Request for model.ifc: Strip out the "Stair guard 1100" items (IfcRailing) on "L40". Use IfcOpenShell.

First a look at what the model holds.

```python
import ifcopenshell
import ifcopenshell.util.element

model = ifcopenshell.open("model.ifc")
print(model.schema)
storey = next(s for s in model.by_type("IfcBuildingStorey") if s.Name == "L40")
railings = [e for e in ifcopenshell.util.element.get_decomposition(storey) if e.is_a("IfcRailing")]
seen = {}
for e in railings:
    element_type = ifcopenshell.util.element.get_type(e)
    name = element_type.Name if element_type not in (None, e) else None
    seen[name] = seen.get(name, 0) + 1
for name, count in sorted(seen.items(), key=str):
    print(count, "x", name)
```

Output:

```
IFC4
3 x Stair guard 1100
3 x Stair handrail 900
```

```python
import ifcopenshell
import ifcopenshell.api.root
import ifcopenshell.util.element

model = ifcopenshell.open("model.ifc")

storey = next(s for s in model.by_type("IfcBuildingStorey") if s.Name == "L40")
railings = [e for e in ifcopenshell.util.element.get_decomposition(storey) if e.is_a("IfcRailing")]
targets = [e for e in railings if (t := ifcopenshell.util.element.get_type(e)) not in (None, e) and t.Name == "Stair guard 1100"]

for e in targets:
    ifcopenshell.api.root.remove_product(model, product=e)
print(len(targets), "removed")

model.write("model_rev.ifc")
```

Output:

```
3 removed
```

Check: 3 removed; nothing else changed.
